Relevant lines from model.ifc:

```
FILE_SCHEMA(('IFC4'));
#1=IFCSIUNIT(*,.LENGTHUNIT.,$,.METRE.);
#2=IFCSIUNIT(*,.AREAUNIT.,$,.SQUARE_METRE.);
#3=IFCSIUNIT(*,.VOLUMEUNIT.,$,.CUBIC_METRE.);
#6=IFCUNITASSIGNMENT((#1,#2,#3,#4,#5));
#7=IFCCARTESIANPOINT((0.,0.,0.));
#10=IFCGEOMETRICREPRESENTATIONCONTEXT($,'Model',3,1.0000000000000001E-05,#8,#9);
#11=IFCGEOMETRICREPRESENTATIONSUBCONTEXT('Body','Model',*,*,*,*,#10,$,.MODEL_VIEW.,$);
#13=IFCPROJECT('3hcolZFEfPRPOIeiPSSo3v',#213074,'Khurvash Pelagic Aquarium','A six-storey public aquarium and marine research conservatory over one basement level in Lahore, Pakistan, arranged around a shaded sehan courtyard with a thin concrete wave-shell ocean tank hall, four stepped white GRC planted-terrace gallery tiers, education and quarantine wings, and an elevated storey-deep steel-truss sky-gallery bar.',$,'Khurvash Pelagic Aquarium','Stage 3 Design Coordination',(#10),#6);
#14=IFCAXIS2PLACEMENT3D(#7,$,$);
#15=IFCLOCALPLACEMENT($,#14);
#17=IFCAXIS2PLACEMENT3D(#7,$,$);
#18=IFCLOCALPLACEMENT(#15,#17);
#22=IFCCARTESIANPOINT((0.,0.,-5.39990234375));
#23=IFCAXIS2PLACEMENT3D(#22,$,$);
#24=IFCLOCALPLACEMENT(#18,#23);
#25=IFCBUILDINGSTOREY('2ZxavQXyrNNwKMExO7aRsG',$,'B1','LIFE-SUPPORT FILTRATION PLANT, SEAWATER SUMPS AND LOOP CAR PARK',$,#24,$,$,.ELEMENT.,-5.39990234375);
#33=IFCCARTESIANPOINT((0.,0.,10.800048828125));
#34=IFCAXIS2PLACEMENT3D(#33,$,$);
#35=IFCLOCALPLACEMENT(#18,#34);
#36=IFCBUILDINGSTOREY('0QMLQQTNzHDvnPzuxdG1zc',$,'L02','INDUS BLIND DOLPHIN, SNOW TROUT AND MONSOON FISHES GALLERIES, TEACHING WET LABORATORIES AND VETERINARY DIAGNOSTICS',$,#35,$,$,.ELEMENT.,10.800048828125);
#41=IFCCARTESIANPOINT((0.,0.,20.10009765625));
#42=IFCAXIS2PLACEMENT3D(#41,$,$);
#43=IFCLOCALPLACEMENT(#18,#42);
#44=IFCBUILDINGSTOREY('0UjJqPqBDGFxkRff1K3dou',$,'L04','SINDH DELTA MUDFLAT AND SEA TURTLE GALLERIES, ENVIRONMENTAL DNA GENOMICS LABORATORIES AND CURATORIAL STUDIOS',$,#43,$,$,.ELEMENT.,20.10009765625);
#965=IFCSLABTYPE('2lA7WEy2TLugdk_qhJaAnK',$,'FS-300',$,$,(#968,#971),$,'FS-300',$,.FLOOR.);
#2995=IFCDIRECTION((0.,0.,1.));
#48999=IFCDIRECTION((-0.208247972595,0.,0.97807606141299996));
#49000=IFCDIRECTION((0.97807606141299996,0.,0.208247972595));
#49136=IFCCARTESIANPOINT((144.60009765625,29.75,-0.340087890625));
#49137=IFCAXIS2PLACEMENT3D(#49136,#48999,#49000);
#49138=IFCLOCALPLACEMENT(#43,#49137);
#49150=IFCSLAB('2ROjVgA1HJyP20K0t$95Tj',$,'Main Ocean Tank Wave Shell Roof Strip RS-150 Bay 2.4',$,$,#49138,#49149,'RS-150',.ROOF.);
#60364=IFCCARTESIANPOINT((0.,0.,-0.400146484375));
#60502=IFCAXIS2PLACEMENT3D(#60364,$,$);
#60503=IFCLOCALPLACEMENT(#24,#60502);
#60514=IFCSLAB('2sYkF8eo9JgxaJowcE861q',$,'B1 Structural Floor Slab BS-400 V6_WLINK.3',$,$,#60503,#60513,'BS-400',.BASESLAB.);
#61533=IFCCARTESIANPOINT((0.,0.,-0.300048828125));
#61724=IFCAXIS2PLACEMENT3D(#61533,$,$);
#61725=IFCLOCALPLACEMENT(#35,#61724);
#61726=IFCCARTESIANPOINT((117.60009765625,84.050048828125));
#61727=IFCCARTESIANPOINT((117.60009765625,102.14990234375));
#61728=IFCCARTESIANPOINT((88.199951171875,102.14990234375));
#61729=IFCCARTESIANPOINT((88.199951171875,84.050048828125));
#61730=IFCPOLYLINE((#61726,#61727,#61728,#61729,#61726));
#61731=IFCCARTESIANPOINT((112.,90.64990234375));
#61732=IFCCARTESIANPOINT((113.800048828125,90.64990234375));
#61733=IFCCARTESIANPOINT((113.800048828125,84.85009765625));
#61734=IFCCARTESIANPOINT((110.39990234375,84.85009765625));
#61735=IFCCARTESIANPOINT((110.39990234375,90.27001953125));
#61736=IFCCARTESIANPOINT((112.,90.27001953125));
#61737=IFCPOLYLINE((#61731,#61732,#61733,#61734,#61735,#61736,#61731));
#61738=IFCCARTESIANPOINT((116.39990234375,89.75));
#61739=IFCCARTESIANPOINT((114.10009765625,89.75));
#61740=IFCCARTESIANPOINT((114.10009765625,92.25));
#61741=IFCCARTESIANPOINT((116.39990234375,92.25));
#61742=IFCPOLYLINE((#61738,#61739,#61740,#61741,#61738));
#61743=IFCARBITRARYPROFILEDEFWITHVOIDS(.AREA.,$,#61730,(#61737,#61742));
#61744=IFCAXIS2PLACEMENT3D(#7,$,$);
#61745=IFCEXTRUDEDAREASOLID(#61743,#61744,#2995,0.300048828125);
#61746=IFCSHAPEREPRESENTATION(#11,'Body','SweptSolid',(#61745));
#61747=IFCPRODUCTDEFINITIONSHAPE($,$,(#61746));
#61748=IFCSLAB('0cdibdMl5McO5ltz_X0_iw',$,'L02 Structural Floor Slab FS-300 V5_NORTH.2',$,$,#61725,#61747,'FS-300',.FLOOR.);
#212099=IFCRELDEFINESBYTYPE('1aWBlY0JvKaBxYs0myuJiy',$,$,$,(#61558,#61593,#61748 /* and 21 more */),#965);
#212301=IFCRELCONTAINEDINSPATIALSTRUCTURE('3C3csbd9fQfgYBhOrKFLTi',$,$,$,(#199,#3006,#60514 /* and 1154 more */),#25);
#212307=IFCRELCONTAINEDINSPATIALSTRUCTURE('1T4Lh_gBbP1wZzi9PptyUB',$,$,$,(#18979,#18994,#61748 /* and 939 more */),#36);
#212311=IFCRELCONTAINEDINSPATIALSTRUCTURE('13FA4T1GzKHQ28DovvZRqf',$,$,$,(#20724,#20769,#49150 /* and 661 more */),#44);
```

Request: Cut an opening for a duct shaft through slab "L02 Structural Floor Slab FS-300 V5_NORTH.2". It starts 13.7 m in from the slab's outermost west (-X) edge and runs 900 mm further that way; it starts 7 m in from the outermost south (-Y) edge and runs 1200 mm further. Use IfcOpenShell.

```python
import numpy as np
import ifcopenshell
import ifcopenshell.api.feature
import ifcopenshell.api.geometry
import ifcopenshell.api.root
import ifcopenshell.geom
import ifcopenshell.util.placement
import ifcopenshell.util.representation
import ifcopenshell.util.shape
import ifcopenshell.util.unit

model = ifcopenshell.open("model.ifc")
unit_scale = ifcopenshell.util.unit.calculate_unit_scale(model)
settings = ifcopenshell.geom.settings()


def volume(element):
    """Net volume in cubic metres, openings subtracted."""
    shape = ifcopenshell.geom.create_shape(settings, element)
    return ifcopenshell.util.shape.get_volume(shape.geometry)


slab = model.by_guid("0cdibdMl5McO5ltz_X0_iw")
before = volume(slab)

# Extent in the slab's own axes, in metres. The edges named are its -X and -Y sides.
slab_shape = ifcopenshell.geom.create_shape(settings, slab)
vertices = ifcopenshell.util.shape.get_vertices(slab_shape.geometry)
x_min, y_min, bottom = vertices.min(axis=0)
top = vertices[:, 2].max()

opening = ifcopenshell.api.root.create_entity(model, ifc_class="IfcOpeningElement", name="Duct shaft opening", predefined_type="OPENING")
context = ifcopenshell.util.representation.get_context(model, "Model", "Body", "MODEL_VIEW")
width, depth = 0.9, 1.2
outline = [(0.0, 0.0), (width, 0.0), (width, depth), (0.0, depth), (0.0, 0.0)]
# Overshoot both faces by 50 mm so the cut is clean.
shape = ifcopenshell.api.geometry.add_slab_representation(
    model, context=context, depth=top - bottom + 0.1, polyline=outline
)
ifcopenshell.api.geometry.assign_representation(model, product=opening, representation=shape)

matrix = ifcopenshell.util.placement.get_local_placement(slab.ObjectPlacement)
matrix[:, 3] = matrix @ np.append(np.array([x_min + 13.7, y_min + 7, bottom - 0.05]) / unit_scale, 1.0)
ifcopenshell.api.geometry.edit_object_placement(model, product=opening, matrix=matrix, is_si=False)
ifcopenshell.api.feature.add_feature(model, feature=opening, element=slab)

after = volume(slab)

print(f"slab volume {before:.3f} -> {after:.3f} m3")

model.write("model-out.ifc")
```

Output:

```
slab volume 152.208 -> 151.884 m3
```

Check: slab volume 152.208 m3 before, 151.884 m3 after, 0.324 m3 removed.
